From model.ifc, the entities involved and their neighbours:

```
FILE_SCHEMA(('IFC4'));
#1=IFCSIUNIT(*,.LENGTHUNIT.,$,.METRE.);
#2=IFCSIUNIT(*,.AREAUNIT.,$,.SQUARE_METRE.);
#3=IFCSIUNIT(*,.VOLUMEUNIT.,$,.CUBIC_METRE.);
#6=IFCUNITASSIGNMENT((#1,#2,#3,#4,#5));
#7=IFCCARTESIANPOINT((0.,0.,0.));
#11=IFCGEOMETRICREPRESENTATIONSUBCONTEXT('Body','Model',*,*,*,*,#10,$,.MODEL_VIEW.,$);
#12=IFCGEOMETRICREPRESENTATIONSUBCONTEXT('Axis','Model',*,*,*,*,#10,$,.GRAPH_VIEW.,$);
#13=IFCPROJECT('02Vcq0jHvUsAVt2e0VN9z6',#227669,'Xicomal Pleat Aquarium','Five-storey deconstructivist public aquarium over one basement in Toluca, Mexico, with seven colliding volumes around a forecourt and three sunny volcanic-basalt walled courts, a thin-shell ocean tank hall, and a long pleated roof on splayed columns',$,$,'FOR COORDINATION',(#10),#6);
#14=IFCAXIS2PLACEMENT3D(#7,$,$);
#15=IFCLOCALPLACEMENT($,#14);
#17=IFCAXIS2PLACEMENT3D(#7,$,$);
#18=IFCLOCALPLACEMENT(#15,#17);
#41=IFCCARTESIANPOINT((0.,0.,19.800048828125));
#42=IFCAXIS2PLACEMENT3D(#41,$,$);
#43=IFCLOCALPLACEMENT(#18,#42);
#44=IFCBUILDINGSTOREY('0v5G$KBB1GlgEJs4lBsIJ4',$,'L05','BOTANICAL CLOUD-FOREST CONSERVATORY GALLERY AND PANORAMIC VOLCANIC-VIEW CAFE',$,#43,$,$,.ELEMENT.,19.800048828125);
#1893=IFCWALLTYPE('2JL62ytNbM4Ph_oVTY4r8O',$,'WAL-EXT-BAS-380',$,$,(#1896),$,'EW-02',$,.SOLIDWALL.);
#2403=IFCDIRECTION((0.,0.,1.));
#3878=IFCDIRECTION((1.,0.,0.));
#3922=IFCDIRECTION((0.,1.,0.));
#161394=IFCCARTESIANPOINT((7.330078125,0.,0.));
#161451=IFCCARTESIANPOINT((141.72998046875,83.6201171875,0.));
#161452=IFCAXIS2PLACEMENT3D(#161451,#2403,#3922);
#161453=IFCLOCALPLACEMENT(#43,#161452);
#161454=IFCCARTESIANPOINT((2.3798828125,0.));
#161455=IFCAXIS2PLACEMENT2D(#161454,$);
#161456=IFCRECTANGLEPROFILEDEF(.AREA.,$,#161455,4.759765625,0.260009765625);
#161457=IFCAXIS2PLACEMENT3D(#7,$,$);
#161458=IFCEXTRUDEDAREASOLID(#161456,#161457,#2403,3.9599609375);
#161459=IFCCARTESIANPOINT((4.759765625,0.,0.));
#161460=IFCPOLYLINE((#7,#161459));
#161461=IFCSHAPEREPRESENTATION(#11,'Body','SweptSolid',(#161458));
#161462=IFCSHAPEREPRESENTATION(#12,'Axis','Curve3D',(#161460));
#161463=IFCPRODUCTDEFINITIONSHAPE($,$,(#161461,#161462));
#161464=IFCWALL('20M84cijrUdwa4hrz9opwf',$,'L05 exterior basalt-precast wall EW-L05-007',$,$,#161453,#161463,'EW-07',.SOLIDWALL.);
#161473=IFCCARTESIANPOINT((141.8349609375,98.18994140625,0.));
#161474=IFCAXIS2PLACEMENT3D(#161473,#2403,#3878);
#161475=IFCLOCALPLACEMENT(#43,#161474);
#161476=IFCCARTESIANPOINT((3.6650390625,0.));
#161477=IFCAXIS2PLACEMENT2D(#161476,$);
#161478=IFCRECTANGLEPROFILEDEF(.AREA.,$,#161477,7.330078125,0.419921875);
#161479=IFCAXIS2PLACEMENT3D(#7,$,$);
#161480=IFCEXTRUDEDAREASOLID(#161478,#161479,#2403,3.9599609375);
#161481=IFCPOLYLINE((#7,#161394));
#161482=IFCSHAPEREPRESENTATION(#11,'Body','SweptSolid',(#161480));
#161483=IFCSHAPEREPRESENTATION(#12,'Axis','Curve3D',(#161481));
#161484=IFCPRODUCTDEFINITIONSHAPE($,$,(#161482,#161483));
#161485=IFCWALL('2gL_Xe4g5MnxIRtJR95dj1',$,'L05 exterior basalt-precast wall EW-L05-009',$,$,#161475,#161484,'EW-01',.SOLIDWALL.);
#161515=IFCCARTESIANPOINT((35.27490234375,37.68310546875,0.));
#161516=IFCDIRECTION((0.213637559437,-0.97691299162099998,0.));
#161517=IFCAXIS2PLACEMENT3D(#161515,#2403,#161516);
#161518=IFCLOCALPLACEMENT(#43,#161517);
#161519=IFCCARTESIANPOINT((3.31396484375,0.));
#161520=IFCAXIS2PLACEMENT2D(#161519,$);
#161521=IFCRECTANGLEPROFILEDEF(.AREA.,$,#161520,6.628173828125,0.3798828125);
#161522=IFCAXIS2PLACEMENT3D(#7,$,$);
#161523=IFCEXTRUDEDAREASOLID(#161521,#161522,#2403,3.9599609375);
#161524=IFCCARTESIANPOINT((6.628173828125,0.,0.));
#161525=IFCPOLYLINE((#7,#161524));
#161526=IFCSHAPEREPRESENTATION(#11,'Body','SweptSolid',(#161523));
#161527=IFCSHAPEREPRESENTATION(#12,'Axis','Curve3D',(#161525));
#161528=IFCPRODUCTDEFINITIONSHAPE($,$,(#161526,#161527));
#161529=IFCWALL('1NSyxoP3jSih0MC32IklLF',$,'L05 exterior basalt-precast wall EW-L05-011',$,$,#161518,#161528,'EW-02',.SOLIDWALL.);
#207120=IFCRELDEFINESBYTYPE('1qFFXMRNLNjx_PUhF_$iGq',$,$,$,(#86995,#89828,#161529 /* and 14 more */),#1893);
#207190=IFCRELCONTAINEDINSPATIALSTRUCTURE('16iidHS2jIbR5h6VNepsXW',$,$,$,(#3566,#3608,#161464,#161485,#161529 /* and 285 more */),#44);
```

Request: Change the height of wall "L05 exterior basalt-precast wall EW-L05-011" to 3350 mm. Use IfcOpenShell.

```python
import ifcopenshell
import ifcopenshell.geom
import ifcopenshell.util.representation
import ifcopenshell.util.shape

model = ifcopenshell.open("model.ifc")
settings = ifcopenshell.geom.settings()


def volume(element):
    """Net volume in cubic metres, openings subtracted."""
    shape = ifcopenshell.geom.create_shape(settings, element)
    return ifcopenshell.util.shape.get_volume(shape.geometry)


wall = model.by_guid("1NSyxoP3jSih0MC32IklLF")
before = volume(wall)

body = ifcopenshell.util.representation.get_representation(wall, "Model", "Body")
solid = body.Items[0]
old_height = solid.Depth
solid.Depth = 3.35
after = volume(wall)

print(f"height {old_height:g} -> {solid.Depth:g}, volume {before:.3f} -> {after:.3f} m3")

model.write("model-out.ifc")
```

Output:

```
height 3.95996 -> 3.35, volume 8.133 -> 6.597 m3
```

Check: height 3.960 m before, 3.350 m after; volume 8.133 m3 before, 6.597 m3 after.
